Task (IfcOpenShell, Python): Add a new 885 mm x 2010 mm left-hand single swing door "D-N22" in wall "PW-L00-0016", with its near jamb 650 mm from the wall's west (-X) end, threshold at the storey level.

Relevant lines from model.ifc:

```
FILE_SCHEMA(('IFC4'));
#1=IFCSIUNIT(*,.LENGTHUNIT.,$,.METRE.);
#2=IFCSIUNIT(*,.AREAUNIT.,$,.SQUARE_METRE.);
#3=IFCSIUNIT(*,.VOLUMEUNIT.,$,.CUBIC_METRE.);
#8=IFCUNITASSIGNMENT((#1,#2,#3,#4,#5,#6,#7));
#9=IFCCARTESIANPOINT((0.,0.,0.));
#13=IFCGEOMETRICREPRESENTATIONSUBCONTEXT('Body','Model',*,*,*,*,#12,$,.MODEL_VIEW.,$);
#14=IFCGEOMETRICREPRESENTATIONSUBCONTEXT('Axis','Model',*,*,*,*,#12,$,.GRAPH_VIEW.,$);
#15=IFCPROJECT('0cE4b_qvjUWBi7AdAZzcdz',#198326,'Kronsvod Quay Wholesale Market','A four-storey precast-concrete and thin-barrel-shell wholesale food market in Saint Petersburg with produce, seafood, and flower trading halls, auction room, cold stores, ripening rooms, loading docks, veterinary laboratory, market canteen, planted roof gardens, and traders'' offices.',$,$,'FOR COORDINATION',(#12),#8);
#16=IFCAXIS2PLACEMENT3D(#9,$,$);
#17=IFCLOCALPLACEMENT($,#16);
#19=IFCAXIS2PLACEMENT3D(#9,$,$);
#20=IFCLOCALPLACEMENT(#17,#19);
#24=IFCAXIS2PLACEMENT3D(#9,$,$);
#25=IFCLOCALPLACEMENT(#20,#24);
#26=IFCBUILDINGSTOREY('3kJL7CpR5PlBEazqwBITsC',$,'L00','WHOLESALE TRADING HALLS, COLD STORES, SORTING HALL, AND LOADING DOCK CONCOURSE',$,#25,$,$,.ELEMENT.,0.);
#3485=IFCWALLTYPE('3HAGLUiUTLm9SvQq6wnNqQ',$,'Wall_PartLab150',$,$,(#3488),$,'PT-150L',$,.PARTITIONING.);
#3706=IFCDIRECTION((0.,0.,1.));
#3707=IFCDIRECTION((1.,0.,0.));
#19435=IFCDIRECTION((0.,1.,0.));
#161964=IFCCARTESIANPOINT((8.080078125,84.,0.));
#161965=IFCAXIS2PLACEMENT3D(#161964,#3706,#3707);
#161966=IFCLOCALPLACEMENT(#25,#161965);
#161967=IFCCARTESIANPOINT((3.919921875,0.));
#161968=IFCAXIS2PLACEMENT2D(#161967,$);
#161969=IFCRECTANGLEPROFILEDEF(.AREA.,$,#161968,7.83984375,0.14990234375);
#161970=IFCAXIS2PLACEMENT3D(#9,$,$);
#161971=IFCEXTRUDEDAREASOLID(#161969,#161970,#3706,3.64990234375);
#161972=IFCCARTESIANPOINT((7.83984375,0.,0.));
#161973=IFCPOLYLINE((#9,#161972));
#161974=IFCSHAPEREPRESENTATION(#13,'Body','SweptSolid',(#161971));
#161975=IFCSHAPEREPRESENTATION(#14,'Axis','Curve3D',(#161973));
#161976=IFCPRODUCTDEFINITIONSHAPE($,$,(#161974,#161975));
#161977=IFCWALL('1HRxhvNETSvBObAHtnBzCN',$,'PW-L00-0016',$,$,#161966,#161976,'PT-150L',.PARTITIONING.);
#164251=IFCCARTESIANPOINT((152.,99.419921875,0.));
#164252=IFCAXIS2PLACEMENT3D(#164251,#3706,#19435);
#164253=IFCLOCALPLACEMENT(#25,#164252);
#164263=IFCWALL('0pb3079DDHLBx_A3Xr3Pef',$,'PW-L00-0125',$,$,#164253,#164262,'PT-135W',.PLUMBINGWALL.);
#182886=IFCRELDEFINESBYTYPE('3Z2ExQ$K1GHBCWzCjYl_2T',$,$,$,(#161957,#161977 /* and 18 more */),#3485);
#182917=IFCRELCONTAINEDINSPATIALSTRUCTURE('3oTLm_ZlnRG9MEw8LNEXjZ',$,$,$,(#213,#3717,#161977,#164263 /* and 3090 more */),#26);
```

```python
import numpy as np
import ifcopenshell
import ifcopenshell.api.feature
import ifcopenshell.api.geometry
import ifcopenshell.api.root
import ifcopenshell.api.spatial
import ifcopenshell.geom
import ifcopenshell.util.element
import ifcopenshell.util.placement
import ifcopenshell.util.representation
import ifcopenshell.util.shape
import ifcopenshell.util.unit

model = ifcopenshell.open("model.ifc")
unit_scale = ifcopenshell.util.unit.calculate_unit_scale(model)
settings = ifcopenshell.geom.settings()


def volume(element):
    """Net volume in cubic metres, openings subtracted."""
    shape = ifcopenshell.geom.create_shape(settings, element)
    return ifcopenshell.util.shape.get_volume(shape.geometry)


wall = model.by_id(161977)
storey = ifcopenshell.util.element.get_container(wall, ifc_class="IfcBuildingStorey")
context = ifcopenshell.util.representation.get_context(model, "Model", "Body", "MODEL_VIEW")
before = volume(wall)

width, height, from_end, sill = 0.885, 2.01, 0.65, 0.0  # metres

# The wall runs along its own X axis, and the end named is its -X end.
wall_shape = ifcopenshell.geom.create_shape(settings, wall)
x, y, z = ifcopenshell.util.shape.get_vertices(wall_shape.geometry).T
start = x.min() + from_end
face, thickness = float(y.min()), float(y.max() - y.min())
wall_matrix = ifcopenshell.util.placement.get_local_placement(wall.ObjectPlacement)
level = ifcopenshell.util.placement.get_local_placement(storey.ObjectPlacement)[2, 3]


def in_wall(x, y):
    """Placement at x, y metres in the wall's axes, at sill height."""
    matrix = wall_matrix.copy()
    matrix[:, 3] = wall_matrix @ np.array([x / unit_scale, y / unit_scale, 0.0, 1.0])
    matrix[2, 3] = level + sill / unit_scale
    return matrix


# Opening: a box that overshoots both wall faces by 50 mm.
opening = ifcopenshell.api.root.create_entity(model, ifc_class="IfcOpeningElement", predefined_type="OPENING")
box = ifcopenshell.api.geometry.add_wall_representation(
    model, context=context, length=width, height=height, thickness=thickness + 0.1
)
ifcopenshell.api.geometry.assign_representation(model, product=opening, representation=box)
ifcopenshell.api.geometry.edit_object_placement(model, product=opening, matrix=in_wall(start, face - 0.05), is_si=False)
ifcopenshell.api.feature.add_feature(model, feature=opening, element=wall)

door = ifcopenshell.api.root.create_entity(model, ifc_class="IfcDoor", name="D-N22", predefined_type="DOOR")
door.OverallWidth, door.OverallHeight = width / unit_scale, height / unit_scale
door.OperationType = "SINGLE_SWING_LEFT"
body = ifcopenshell.api.geometry.add_door_representation(
    model,
    context=context,
    overall_width=door.OverallWidth,
    overall_height=door.OverallHeight,
    operation_type="SINGLE_SWING_LEFT",
    lining_properties={"LiningDepth": thickness / unit_scale, "ThresholdDepth": thickness / unit_scale},
)
ifcopenshell.api.geometry.assign_representation(model, product=door, representation=body)
ifcopenshell.api.spatial.assign_container(model, products=[door], relating_structure=storey)
ifcopenshell.api.feature.add_filling(model, opening=opening, element=door)

# The lining spans the wall, so the door starts at the wall face.
ifcopenshell.api.geometry.edit_object_placement(model, product=door, matrix=in_wall(start, face), is_si=False)

after = volume(wall)

print(f"wall volume {before:.3f} -> {after:.3f} m3")

model.write("model-out.ifc")
```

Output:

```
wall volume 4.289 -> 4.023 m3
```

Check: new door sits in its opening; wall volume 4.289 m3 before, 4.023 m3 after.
